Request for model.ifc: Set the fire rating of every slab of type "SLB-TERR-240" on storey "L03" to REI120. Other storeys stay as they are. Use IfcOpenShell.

First a look at what the model holds.

```python
import ifcopenshell
import ifcopenshell.util.element

model = ifcopenshell.open("model.ifc")
print(model.schema)
storey = next(s for s in model.by_type("IfcBuildingStorey") if s.Name == "L03")
slabs = [e for e in ifcopenshell.util.element.get_decomposition(storey) if e.is_a("IfcSlab")]
seen = {}
for e in slabs:
    element_type = ifcopenshell.util.element.get_type(e)
    key = (element_type.Name if element_type != e and element_type else None, ifcopenshell.util.element.get_pset(e, "Pset_SlabCommon", "FireRating"))
    seen[key] = seen.get(key, 0) + 1
for (name, value), count in sorted(seen.items(), key=str):
    print(count, "x", name, "|", value)
```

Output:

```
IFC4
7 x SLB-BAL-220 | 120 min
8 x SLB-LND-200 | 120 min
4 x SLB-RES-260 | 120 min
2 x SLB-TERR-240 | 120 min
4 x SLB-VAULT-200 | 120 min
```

```python
import ifcopenshell
import ifcopenshell.api.pset
import ifcopenshell.util.element

model = ifcopenshell.open("model.ifc")

storey = next(s for s in model.by_type("IfcBuildingStorey") if s.Name == "L03")
slabs = [e for e in ifcopenshell.util.element.get_decomposition(storey) if e.is_a("IfcSlab")]

count = 0
for e in slabs:
    element_type = ifcopenshell.util.element.get_type(e)
    if element_type in (None, e) or element_type.Name != "SLB-TERR-240":
        continue
    # add_pset returns the element's existing set when there is one.
    pset = ifcopenshell.api.pset.add_pset(model, product=e, name="Pset_SlabCommon")
    ifcopenshell.api.pset.edit_pset(model, pset=pset, properties={"FireRating": "REI120"})
    count += 1

print(count, "slabs updated")

model.write("model_updated.ifc")
```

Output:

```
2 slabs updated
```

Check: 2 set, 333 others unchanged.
